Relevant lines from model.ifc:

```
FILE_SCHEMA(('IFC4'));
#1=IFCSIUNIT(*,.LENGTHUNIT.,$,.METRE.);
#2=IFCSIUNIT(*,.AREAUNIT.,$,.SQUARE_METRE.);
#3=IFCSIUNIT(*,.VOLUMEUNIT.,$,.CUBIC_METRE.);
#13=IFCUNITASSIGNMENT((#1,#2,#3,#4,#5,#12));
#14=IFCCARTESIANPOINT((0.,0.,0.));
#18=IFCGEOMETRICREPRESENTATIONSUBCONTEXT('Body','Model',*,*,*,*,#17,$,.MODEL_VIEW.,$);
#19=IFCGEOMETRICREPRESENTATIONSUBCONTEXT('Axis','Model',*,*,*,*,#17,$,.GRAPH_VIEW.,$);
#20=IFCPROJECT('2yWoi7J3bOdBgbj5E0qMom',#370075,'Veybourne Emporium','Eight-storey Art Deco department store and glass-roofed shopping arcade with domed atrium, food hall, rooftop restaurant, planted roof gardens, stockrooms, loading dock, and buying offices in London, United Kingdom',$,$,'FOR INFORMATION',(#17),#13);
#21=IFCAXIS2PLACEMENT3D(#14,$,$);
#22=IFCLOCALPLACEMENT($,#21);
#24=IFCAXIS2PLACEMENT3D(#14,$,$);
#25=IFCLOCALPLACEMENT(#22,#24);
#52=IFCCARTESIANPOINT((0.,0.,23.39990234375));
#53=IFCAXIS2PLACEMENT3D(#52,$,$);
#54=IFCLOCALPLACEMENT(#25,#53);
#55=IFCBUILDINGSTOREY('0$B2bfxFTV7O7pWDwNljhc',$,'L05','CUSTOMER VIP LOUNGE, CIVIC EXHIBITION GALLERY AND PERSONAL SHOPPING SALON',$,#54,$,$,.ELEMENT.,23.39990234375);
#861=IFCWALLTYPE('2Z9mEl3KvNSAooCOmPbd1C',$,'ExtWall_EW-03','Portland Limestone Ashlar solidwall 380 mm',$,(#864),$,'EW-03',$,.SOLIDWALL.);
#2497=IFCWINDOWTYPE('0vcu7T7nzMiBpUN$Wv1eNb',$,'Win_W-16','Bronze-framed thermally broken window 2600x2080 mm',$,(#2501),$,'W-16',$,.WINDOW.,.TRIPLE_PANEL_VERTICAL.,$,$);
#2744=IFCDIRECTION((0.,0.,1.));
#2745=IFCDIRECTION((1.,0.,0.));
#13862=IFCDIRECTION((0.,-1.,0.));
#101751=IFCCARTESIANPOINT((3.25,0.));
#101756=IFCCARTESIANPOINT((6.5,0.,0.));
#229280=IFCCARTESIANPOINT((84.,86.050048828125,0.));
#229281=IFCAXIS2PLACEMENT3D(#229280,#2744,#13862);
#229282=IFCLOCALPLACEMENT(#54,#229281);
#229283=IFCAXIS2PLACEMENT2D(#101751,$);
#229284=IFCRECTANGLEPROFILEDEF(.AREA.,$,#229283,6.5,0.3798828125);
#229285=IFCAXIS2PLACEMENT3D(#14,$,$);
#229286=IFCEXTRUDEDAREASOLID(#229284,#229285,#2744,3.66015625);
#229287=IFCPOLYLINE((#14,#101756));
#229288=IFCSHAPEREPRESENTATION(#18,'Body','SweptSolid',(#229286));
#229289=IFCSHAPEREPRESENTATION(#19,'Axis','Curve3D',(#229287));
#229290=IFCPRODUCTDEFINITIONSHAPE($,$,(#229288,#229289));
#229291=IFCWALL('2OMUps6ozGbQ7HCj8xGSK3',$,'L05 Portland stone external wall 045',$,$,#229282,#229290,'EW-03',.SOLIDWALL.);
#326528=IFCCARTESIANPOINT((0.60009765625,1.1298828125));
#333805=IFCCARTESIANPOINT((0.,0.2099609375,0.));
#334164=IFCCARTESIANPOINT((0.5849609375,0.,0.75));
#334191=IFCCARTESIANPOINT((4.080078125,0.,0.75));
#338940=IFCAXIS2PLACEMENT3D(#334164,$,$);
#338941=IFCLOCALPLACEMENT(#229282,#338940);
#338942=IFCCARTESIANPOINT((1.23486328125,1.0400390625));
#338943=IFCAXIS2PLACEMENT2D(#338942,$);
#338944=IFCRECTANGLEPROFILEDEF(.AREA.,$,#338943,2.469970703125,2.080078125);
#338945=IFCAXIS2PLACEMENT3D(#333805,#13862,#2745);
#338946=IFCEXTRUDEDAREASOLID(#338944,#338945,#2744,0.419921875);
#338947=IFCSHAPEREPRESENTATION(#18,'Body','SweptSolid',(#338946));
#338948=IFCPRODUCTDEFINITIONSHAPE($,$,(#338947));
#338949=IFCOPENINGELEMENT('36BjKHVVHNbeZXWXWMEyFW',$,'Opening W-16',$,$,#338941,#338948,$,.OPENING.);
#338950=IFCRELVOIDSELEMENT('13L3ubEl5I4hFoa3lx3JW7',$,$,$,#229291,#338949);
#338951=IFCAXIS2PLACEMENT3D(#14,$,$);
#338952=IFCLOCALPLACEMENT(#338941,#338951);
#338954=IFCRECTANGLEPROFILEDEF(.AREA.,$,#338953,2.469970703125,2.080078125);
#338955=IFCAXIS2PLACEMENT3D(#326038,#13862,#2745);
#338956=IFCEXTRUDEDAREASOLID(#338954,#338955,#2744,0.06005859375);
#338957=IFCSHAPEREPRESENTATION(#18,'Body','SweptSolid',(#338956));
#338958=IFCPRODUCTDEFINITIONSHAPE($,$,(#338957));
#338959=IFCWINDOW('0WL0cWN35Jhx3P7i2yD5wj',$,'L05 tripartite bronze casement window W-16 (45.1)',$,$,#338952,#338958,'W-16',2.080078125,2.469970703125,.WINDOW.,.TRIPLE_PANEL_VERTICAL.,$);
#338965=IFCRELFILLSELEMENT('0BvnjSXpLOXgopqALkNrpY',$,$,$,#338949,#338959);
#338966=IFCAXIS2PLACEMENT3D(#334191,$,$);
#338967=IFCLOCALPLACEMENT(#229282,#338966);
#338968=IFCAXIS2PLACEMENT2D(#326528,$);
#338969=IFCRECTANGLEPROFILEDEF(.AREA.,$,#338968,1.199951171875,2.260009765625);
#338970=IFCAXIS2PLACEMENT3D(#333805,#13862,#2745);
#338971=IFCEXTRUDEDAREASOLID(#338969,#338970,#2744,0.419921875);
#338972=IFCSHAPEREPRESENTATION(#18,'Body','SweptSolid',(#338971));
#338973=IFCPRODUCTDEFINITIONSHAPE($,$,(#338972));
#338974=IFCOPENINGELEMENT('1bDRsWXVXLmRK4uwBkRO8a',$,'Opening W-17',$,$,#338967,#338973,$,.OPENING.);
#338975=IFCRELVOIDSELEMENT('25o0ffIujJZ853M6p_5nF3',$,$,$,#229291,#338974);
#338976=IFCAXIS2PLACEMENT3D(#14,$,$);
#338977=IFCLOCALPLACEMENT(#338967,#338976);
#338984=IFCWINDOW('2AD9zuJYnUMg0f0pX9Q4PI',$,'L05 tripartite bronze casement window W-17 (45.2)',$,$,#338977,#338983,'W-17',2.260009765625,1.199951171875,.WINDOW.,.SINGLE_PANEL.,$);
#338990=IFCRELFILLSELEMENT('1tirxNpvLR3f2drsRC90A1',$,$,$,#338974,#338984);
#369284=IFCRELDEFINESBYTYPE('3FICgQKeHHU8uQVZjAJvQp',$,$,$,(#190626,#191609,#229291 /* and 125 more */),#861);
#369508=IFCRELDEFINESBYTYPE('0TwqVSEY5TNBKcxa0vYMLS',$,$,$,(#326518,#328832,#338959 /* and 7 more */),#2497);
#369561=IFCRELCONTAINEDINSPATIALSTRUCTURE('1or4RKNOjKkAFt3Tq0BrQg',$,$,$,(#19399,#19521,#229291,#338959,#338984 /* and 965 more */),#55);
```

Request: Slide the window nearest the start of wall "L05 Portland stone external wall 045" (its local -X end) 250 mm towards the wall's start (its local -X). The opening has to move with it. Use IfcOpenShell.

```python
import ifcopenshell
import ifcopenshell.api.geometry
import ifcopenshell.util.placement
import ifcopenshell.util.unit

model = ifcopenshell.open("model.ifc")
unit_scale = ifcopenshell.util.unit.calculate_unit_scale(model)

window = model.by_id(338959)
opening = window.FillsVoids[0].RelatingOpeningElement
wall = opening.VoidsElements[0].RelatingBuildingElement

wall_matrix = ifcopenshell.util.placement.get_local_placement(wall.ObjectPlacement)
shift = wall_matrix[:3, 0] * -0.25 / unit_scale
before = ifcopenshell.util.placement.get_local_placement(window.ObjectPlacement)[:3, 3].copy()

# The window is placed relative to its opening, so it follows when the opening moves.
matrix = ifcopenshell.util.placement.get_local_placement(opening.ObjectPlacement)
matrix[:3, 3] += shift
ifcopenshell.api.geometry.edit_object_placement(
    model, product=opening, matrix=matrix, is_si=False, should_transform_children=True
)

after = ifcopenshell.util.placement.get_local_placement(window.ObjectPlacement)[:3, 3]
print("window moved by", (after - before).round(3) + 0.0)

model.write("model_rev.ifc")
```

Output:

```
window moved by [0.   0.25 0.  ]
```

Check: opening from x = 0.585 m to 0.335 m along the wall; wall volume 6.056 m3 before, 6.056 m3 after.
